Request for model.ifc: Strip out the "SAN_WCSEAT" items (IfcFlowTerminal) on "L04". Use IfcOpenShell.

First a look at what the model holds.

```python
import ifcopenshell
import ifcopenshell.util.element

model = ifcopenshell.open("model.ifc")
print(model.schema)
storey = next(s for s in model.by_type("IfcBuildingStorey") if s.Name == "L04")
terminals = [e for e in ifcopenshell.util.element.get_decomposition(storey) if e.is_a("IfcFlowTerminal")]
seen = {}
for e in terminals:
    element_type = ifcopenshell.util.element.get_type(e)
    name = element_type.Name if element_type not in (None, e) else None
    seen[name] = seen.get(name, 0) + 1
for name, count in sorted(seen.items(), key=str):
    print(count, "x", name)
```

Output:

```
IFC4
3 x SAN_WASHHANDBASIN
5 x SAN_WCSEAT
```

```python
import ifcopenshell
import ifcopenshell.api.root
import ifcopenshell.util.element

model = ifcopenshell.open("model.ifc")

storey = next(s for s in model.by_type("IfcBuildingStorey") if s.Name == "L04")
terminals = [e for e in ifcopenshell.util.element.get_decomposition(storey) if e.is_a("IfcFlowTerminal")]
targets = [e for e in terminals if (t := ifcopenshell.util.element.get_type(e)) not in (None, e) and t.Name == "SAN_WCSEAT"]

for e in targets:
    ifcopenshell.api.root.remove_product(model, product=e)
print(len(targets), "removed")

model.write("model-out.ifc")
```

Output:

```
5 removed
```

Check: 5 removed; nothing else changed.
